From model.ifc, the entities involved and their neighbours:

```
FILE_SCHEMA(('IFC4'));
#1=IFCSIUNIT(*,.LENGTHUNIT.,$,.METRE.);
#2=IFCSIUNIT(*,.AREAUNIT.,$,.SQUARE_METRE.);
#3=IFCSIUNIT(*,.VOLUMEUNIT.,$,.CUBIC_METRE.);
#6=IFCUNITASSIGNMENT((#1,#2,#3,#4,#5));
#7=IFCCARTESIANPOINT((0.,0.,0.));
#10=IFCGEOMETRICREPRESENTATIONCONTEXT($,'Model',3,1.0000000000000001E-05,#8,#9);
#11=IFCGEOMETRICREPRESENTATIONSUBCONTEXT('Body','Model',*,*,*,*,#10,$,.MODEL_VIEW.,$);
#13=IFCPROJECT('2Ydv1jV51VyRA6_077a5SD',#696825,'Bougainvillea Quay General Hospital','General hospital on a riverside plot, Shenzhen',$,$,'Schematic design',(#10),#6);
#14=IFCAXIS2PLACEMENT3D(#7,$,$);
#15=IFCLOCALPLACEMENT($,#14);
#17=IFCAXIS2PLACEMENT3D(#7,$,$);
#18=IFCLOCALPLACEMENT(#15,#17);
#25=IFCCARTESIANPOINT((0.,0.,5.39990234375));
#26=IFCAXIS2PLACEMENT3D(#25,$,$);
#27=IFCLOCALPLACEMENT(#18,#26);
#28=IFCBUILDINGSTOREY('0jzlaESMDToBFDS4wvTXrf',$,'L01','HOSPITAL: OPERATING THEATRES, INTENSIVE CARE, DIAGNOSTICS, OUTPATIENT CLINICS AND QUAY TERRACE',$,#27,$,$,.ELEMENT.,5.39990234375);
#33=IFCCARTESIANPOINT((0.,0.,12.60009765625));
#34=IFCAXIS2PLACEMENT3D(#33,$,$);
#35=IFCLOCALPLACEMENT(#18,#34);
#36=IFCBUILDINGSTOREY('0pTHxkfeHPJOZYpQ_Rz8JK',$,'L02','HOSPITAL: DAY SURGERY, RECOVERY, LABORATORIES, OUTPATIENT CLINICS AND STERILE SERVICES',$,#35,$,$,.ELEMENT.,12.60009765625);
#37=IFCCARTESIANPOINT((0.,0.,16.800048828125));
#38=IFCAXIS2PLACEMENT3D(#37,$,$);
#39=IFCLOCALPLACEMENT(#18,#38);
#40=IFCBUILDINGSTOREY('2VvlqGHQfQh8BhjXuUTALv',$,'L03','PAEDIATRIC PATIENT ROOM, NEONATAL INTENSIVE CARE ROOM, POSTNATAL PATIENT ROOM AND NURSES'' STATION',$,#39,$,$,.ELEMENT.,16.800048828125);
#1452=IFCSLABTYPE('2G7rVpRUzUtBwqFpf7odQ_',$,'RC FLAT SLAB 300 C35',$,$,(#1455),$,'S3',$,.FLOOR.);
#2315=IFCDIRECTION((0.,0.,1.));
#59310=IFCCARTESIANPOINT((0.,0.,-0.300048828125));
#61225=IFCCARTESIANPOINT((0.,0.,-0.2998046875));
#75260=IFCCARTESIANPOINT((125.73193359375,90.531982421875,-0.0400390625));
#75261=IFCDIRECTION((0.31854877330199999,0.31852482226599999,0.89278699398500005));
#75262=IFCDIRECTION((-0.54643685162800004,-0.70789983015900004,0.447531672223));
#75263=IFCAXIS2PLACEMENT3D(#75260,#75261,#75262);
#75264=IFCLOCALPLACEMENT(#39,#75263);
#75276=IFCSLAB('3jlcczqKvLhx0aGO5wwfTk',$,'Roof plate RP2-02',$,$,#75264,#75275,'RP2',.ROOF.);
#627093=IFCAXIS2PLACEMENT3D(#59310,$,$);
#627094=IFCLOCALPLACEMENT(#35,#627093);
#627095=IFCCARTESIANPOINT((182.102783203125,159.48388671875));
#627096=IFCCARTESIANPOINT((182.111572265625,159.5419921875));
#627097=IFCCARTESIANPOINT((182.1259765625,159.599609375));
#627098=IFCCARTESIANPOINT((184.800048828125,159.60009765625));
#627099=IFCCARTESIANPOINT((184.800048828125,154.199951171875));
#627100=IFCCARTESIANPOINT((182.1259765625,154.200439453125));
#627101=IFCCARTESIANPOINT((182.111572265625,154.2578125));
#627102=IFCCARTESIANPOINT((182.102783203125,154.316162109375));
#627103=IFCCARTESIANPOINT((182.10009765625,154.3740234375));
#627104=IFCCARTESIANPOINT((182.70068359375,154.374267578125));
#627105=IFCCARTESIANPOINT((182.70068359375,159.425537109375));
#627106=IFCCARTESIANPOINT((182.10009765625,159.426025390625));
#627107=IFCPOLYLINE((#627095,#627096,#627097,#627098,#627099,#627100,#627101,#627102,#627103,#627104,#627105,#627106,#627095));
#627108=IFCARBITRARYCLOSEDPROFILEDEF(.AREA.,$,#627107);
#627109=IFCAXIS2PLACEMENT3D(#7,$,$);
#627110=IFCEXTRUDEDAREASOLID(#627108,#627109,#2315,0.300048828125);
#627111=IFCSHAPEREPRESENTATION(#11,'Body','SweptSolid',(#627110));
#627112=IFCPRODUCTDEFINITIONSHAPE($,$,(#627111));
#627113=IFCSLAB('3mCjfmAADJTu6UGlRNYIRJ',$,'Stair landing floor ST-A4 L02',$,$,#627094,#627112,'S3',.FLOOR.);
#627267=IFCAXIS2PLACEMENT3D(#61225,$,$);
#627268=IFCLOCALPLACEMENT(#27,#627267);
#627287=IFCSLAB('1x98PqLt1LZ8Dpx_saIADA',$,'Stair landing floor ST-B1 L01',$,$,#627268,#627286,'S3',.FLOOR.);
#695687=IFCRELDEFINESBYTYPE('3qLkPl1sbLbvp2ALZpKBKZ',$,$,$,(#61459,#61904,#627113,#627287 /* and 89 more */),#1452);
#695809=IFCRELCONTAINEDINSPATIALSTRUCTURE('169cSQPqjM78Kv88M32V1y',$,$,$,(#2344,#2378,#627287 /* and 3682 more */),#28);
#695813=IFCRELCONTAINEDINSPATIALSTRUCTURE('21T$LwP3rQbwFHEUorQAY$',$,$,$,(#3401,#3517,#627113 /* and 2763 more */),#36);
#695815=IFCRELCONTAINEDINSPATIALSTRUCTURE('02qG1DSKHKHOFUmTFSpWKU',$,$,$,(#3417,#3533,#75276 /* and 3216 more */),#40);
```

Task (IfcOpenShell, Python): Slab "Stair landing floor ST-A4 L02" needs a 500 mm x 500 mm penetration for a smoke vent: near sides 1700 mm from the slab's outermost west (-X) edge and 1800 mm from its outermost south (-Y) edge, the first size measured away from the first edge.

```python
import numpy as np
import ifcopenshell
import ifcopenshell.api.feature
import ifcopenshell.api.geometry
import ifcopenshell.api.root
import ifcopenshell.geom
import ifcopenshell.util.placement
import ifcopenshell.util.representation
import ifcopenshell.util.shape
import ifcopenshell.util.unit

model = ifcopenshell.open("model.ifc")
unit_scale = ifcopenshell.util.unit.calculate_unit_scale(model)
settings = ifcopenshell.geom.settings()


def volume(element):
    """Net volume in cubic metres, openings subtracted."""
    shape = ifcopenshell.geom.create_shape(settings, element)
    return ifcopenshell.util.shape.get_volume(shape.geometry)


slab = model.by_guid("3mCjfmAADJTu6UGlRNYIRJ")
before = volume(slab)

# Extent in the slab's own axes, in metres. The edges named are its -X and -Y sides.
slab_shape = ifcopenshell.geom.create_shape(settings, slab)
vertices = ifcopenshell.util.shape.get_vertices(slab_shape.geometry)
x_min, y_min, bottom = vertices.min(axis=0)
top = vertices[:, 2].max()

opening = ifcopenshell.api.root.create_entity(model, ifc_class="IfcOpeningElement", name="Smoke vent opening", predefined_type="OPENING")
context = ifcopenshell.util.representation.get_context(model, "Model", "Body", "MODEL_VIEW")
width, depth = 0.5, 0.5
outline = [(0.0, 0.0), (width, 0.0), (width, depth), (0.0, depth), (0.0, 0.0)]
# Overshoot both faces by 50 mm so the cut is clean.
shape = ifcopenshell.api.geometry.add_slab_representation(
    model, context=context, depth=top - bottom + 0.1, polyline=outline
)
ifcopenshell.api.geometry.assign_representation(model, product=opening, representation=shape)

matrix = ifcopenshell.util.placement.get_local_placement(slab.ObjectPlacement)
matrix[:, 3] = matrix @ np.append(np.array([x_min + 1.7, y_min + 1.8, bottom - 0.05]) / unit_scale, 1.0)
ifcopenshell.api.geometry.edit_object_placement(model, product=opening, matrix=matrix, is_si=False)
ifcopenshell.api.feature.add_feature(model, feature=opening, element=slab)

after = volume(slab)

print(f"slab volume {before:.3f} -> {after:.3f} m3")

model.write("model_rev.ifc")
```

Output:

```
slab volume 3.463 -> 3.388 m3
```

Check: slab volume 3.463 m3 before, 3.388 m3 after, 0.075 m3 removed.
